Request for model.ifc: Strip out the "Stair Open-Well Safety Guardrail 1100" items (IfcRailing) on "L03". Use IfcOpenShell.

First a look at what the model holds.

```python
import ifcopenshell
import ifcopenshell.util.element

model = ifcopenshell.open("model.ifc")
print(model.schema)
storey = next(s for s in model.by_type("IfcBuildingStorey") if s.Name == "L03")
railings = [e for e in ifcopenshell.util.element.get_decomposition(storey) if e.is_a("IfcRailing")]
seen = {}
for e in railings:
    element_type = ifcopenshell.util.element.get_type(e)
    name = element_type.Name if element_type not in (None, e) else None
    seen[name] = seen.get(name, 0) + 1
for name, count in sorted(seen.items(), key=str):
    print(count, "x", name)
```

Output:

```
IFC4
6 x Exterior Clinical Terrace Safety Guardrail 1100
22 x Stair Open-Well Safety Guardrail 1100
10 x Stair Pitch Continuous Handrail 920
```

```python
import ifcopenshell
import ifcopenshell.api.root
import ifcopenshell.util.element

model = ifcopenshell.open("model.ifc")

storey = next(s for s in model.by_type("IfcBuildingStorey") if s.Name == "L03")
railings = [e for e in ifcopenshell.util.element.get_decomposition(storey) if e.is_a("IfcRailing")]
targets = [e for e in railings if (t := ifcopenshell.util.element.get_type(e)) not in (None, e) and t.Name == "Stair Open-Well Safety Guardrail 1100"]

for e in targets:
    ifcopenshell.api.root.remove_product(model, product=e)
print(len(targets), "removed")

model.write("model_edited.ifc")
```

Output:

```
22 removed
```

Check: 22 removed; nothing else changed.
